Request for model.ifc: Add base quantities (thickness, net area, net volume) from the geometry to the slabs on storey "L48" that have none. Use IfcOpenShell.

First a look at what the model holds.

```python
import ifcopenshell
import ifcopenshell.util.element
import ifcopenshell.util.unit

model = ifcopenshell.open("model.ifc")
print(model.schema)
for unit_type in ("LENGTHUNIT", "AREAUNIT", "VOLUMEUNIT"):
    print(unit_type, ifcopenshell.util.unit.calculate_unit_scale(model, unit_type))
storey = next(s for s in model.by_type("IfcBuildingStorey") if s.Name == "L48")
slabs = [e for e in ifcopenshell.util.element.get_decomposition(storey) if e.is_a("IfcSlab")]
for e in sorted(slabs, key=lambda e: e.id()):
    print(e.id(), e.is_a(), e.Name, list(ifcopenshell.util.element.get_psets(e, qtos_only=True)), sep=" | ")
```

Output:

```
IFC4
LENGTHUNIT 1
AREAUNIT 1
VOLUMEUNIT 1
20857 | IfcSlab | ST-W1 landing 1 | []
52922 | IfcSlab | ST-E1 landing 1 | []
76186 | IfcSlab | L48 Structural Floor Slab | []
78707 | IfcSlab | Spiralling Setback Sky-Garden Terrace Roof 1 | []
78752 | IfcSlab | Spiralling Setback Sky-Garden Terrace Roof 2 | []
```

```python
import ifcopenshell
import ifcopenshell.api.pset
import ifcopenshell.geom
import ifcopenshell.util.element
import ifcopenshell.util.shape
import ifcopenshell.util.unit

model = ifcopenshell.open("model.ifc")
unit_scale = ifcopenshell.util.unit.calculate_unit_scale(model)
area_scale = ifcopenshell.util.unit.calculate_unit_scale(model, "AREAUNIT")
volume_scale = ifcopenshell.util.unit.calculate_unit_scale(model, "VOLUMEUNIT")
settings = ifcopenshell.geom.settings()

storey = next(s for s in model.by_type("IfcBuildingStorey") if s.Name == "L48")
slabs = [e for e in ifcopenshell.util.element.get_decomposition(storey) if e.is_a("IfcSlab")]

for e in sorted(slabs, key=lambda e: e.id()):
    if ifcopenshell.util.element.get_psets(e, qtos_only=True, should_inherit=False):
        continue
    # Geometry comes back in metres, in the element's own axes.
    shape = ifcopenshell.geom.create_shape(settings, e)
    values = {
        "Width": ifcopenshell.util.shape.get_z(shape.geometry) / unit_scale,
        "NetArea": ifcopenshell.util.shape.get_footprint_area(shape.geometry) / area_scale,
        "NetVolume": ifcopenshell.util.shape.get_volume(shape.geometry) / volume_scale,
    }
    qto = ifcopenshell.api.pset.add_qto(model, product=e, name="Qto_SlabBaseQuantities")
    ifcopenshell.api.pset.edit_qto(model, qto=qto, properties=values)
    print(e.id(), {k: round(v, 3) for k, v in values.items()})

model.write("model_updated.ifc")
```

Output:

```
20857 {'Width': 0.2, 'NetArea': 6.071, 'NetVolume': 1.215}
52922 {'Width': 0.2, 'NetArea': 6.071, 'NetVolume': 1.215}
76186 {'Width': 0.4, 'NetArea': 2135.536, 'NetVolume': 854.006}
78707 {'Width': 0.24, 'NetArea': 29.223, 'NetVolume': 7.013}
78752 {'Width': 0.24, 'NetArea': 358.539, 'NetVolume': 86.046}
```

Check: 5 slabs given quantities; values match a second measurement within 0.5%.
